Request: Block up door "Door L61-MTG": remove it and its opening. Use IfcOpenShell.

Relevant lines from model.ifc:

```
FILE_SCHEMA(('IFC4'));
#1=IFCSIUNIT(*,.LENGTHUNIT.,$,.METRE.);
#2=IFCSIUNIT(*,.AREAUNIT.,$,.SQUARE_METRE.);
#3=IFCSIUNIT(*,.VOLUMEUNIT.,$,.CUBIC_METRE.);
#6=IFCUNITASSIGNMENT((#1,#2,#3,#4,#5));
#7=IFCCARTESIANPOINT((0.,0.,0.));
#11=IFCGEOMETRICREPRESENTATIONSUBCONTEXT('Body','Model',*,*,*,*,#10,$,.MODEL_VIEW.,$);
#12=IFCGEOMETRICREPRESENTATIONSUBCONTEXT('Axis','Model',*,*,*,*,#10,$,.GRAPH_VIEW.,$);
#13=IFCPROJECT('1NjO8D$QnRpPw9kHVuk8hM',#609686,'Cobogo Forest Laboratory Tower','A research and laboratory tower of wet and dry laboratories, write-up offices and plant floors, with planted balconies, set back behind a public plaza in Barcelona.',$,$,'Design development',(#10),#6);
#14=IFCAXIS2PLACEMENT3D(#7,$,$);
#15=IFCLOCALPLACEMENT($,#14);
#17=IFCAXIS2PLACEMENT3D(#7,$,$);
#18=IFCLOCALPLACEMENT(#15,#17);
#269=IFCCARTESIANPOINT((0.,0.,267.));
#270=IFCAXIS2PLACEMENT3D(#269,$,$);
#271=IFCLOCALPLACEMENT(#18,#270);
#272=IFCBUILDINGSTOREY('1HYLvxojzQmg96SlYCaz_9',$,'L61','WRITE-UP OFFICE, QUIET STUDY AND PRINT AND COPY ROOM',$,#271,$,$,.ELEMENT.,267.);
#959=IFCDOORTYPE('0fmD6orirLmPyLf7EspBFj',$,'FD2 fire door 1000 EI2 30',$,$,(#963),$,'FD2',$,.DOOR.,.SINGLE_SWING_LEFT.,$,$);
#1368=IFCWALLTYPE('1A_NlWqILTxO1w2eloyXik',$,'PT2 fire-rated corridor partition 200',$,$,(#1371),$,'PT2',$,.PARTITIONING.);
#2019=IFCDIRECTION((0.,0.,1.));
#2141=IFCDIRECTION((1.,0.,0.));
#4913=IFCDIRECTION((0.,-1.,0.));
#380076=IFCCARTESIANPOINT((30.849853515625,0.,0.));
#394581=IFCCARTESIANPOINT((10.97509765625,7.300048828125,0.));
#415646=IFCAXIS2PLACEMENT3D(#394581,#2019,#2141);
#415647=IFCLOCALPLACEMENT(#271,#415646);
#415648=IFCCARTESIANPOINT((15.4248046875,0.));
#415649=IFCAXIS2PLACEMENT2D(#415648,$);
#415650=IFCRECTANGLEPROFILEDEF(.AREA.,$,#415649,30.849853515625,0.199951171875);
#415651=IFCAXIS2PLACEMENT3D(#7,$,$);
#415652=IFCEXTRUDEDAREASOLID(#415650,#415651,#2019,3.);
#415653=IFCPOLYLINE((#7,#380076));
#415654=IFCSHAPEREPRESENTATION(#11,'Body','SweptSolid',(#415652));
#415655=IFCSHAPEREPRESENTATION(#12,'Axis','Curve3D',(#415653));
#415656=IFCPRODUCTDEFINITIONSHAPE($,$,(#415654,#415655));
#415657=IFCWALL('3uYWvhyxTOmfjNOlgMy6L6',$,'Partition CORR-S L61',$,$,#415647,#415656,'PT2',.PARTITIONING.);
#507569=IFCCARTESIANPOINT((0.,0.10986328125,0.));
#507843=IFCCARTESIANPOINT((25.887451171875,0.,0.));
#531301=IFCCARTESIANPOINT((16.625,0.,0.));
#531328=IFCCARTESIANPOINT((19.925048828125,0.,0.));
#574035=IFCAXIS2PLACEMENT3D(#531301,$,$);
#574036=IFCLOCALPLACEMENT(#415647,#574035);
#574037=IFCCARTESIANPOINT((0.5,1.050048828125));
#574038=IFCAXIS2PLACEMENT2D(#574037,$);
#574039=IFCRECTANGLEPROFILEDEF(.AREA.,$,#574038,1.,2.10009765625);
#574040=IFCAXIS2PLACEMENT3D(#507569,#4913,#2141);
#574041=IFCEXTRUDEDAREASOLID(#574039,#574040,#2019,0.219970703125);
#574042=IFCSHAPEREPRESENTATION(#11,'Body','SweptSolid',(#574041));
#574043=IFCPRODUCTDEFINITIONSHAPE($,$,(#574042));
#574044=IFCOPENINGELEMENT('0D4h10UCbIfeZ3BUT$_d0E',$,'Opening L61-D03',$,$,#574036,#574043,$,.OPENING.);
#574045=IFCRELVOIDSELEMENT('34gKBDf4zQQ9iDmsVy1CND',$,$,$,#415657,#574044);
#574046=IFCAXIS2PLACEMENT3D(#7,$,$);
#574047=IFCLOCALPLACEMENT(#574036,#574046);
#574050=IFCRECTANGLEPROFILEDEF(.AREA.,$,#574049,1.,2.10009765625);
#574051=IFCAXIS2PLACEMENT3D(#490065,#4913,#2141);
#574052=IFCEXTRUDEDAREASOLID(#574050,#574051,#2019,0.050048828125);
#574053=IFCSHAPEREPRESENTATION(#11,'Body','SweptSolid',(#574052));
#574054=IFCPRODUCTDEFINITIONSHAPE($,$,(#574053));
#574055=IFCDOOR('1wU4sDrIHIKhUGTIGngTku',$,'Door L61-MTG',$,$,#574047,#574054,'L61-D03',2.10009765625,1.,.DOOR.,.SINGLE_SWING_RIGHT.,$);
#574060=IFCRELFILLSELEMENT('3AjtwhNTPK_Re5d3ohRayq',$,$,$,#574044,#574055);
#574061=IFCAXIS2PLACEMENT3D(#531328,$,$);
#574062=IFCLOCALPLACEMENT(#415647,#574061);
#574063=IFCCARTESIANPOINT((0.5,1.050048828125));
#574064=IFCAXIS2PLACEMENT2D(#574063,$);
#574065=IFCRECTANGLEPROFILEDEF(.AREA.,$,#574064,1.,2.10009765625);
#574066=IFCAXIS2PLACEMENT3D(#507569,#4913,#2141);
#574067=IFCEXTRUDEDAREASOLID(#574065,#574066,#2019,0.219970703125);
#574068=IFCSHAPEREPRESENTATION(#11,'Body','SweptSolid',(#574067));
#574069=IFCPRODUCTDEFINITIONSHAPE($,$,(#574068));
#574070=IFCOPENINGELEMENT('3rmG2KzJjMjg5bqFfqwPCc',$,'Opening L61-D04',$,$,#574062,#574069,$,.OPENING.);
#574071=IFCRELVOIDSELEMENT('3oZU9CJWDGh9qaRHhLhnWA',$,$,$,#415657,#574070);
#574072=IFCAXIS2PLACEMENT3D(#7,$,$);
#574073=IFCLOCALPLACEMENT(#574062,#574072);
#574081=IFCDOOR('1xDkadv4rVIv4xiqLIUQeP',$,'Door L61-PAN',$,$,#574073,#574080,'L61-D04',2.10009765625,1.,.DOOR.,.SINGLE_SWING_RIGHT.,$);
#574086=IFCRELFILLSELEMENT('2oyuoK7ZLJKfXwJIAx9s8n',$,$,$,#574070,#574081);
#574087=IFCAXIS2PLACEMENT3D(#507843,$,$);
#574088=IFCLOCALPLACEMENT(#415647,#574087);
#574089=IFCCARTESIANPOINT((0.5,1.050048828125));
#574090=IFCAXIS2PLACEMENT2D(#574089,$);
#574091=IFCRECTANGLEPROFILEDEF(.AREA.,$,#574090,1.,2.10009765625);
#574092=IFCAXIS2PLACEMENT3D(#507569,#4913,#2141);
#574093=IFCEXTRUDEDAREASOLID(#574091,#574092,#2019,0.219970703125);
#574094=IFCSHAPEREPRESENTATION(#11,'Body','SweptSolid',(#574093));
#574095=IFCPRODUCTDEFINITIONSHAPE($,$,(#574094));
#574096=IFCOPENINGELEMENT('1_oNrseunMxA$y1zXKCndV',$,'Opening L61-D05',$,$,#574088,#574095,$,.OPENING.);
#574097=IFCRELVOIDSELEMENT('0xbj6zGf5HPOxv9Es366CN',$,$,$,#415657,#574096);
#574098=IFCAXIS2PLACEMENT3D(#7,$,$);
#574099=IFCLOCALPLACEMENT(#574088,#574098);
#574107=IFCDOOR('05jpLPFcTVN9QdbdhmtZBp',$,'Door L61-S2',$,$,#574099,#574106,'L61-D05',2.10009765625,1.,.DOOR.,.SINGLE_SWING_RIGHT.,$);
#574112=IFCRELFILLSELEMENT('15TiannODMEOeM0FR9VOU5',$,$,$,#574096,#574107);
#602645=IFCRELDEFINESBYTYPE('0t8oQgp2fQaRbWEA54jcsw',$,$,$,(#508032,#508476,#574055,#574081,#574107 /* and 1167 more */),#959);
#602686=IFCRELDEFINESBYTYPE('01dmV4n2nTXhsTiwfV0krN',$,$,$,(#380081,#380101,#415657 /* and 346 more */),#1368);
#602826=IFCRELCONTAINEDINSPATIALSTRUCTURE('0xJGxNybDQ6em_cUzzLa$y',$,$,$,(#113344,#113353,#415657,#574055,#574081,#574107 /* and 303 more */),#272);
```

```python
import ifcopenshell
import ifcopenshell.api.feature
import ifcopenshell.api.root
import ifcopenshell.geom
import ifcopenshell.util.shape

model = ifcopenshell.open("model.ifc")
settings = ifcopenshell.geom.settings()


def volume(element):
    """Net volume in cubic metres, openings subtracted."""
    shape = ifcopenshell.geom.create_shape(settings, element)
    return ifcopenshell.util.shape.get_volume(shape.geometry)


door = model.by_guid("1wU4sDrIHIKhUGTIGngTku")
opening = door.FillsVoids[0].RelatingOpeningElement
wall = opening.VoidsElements[0].RelatingBuildingElement
before = volume(wall)

ifcopenshell.api.root.remove_product(model, product=door)
ifcopenshell.api.feature.remove_feature(model, feature=opening)

after = volume(wall)

print(f"wall volume {before:.3f} -> {after:.3f} m3")

model.write("model_edited.ifc")
```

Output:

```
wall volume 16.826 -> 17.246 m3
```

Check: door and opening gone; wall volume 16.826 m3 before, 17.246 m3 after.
